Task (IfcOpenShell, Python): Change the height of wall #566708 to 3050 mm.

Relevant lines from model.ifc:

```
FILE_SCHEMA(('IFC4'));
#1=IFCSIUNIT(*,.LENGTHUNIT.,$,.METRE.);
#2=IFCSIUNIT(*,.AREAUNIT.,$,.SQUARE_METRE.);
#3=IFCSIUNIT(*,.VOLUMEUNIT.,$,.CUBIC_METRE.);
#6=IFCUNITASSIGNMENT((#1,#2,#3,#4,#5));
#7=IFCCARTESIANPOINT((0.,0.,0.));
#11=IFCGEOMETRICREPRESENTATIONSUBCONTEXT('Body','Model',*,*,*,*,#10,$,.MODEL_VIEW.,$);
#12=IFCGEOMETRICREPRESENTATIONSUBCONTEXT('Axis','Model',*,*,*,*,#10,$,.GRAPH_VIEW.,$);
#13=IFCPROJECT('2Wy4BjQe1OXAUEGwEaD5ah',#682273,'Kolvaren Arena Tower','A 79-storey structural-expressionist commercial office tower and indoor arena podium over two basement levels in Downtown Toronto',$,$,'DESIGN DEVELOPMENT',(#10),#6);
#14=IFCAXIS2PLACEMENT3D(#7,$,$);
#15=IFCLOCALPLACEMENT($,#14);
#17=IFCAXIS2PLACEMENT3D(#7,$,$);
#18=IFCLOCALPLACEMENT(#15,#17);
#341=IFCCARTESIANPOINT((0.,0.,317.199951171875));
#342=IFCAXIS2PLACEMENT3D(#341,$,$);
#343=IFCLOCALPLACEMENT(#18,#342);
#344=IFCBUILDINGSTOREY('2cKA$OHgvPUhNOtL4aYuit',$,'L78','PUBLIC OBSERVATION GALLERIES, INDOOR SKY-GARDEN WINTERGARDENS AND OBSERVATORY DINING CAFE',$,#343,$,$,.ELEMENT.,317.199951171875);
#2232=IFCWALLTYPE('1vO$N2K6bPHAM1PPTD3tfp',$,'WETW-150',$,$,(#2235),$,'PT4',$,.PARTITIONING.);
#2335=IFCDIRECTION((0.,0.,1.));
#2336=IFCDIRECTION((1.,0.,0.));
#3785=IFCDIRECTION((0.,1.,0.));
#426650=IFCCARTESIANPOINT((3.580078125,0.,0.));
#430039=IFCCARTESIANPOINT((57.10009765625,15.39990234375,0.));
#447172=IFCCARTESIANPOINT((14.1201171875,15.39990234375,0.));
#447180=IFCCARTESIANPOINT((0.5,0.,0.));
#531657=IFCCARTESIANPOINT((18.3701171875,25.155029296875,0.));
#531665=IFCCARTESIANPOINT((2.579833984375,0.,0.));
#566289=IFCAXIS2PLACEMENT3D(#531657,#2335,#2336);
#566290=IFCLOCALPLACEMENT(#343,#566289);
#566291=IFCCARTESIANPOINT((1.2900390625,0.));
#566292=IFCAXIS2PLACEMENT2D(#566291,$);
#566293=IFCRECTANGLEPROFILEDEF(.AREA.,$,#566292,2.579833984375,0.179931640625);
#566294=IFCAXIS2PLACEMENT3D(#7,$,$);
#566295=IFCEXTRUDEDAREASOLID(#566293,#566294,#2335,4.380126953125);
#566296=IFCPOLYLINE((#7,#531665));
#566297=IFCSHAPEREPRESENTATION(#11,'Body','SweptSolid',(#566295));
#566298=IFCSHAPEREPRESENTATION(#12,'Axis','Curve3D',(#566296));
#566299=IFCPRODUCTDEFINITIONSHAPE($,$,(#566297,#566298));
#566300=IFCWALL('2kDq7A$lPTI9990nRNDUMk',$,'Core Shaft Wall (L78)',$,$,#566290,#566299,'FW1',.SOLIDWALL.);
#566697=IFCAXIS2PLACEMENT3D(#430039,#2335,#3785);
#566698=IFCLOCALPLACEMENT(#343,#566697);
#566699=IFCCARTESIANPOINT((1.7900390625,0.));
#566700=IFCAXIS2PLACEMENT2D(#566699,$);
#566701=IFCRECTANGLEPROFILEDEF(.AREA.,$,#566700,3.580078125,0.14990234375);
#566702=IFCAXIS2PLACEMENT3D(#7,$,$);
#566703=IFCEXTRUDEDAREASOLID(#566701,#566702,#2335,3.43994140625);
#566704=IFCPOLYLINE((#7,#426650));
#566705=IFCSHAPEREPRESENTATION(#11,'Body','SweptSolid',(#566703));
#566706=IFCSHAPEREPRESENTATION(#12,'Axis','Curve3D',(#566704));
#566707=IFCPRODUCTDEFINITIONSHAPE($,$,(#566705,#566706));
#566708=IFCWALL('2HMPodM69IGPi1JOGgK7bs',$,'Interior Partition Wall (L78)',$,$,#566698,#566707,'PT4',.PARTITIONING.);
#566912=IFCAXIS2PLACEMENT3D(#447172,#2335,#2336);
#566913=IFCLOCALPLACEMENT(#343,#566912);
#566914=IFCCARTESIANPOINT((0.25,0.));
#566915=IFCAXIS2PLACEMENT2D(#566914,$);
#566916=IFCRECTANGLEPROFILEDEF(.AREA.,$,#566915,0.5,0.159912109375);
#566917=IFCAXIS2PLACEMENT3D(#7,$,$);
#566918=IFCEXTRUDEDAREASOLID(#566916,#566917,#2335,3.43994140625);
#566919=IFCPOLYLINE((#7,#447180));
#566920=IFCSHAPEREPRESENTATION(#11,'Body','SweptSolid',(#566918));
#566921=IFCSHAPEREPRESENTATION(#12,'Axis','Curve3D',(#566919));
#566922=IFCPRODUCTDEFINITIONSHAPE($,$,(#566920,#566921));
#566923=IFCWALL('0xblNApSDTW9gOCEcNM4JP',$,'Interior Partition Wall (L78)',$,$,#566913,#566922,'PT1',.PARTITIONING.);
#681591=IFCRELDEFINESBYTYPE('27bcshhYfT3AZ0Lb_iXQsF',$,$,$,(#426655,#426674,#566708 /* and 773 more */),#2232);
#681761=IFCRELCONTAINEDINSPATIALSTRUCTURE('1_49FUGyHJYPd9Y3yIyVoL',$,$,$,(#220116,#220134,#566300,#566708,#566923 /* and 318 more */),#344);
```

```python
import ifcopenshell
import ifcopenshell.geom
import ifcopenshell.util.representation
import ifcopenshell.util.shape
import ifcopenshell.util.unit

model = ifcopenshell.open("model.ifc")
unit_scale = ifcopenshell.util.unit.calculate_unit_scale(model)
settings = ifcopenshell.geom.settings()


def volume(element):
    """Net volume in cubic metres, openings subtracted."""
    shape = ifcopenshell.geom.create_shape(settings, element)
    return ifcopenshell.util.shape.get_volume(shape.geometry)


wall = model.by_guid("2HMPodM69IGPi1JOGgK7bs")
before = volume(wall)

body = ifcopenshell.util.representation.get_representation(wall, "Model", "Body")
solid = body.Items[0]
old_height = solid.Depth
solid.Depth = 3.05 / unit_scale
after = volume(wall)

print(f"height {old_height:g} -> {solid.Depth:g}, volume {before:.3f} -> {after:.3f} m3")

model.write("model-out.ifc")
```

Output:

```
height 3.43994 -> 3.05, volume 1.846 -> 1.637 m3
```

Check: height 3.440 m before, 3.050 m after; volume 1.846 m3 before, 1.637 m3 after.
